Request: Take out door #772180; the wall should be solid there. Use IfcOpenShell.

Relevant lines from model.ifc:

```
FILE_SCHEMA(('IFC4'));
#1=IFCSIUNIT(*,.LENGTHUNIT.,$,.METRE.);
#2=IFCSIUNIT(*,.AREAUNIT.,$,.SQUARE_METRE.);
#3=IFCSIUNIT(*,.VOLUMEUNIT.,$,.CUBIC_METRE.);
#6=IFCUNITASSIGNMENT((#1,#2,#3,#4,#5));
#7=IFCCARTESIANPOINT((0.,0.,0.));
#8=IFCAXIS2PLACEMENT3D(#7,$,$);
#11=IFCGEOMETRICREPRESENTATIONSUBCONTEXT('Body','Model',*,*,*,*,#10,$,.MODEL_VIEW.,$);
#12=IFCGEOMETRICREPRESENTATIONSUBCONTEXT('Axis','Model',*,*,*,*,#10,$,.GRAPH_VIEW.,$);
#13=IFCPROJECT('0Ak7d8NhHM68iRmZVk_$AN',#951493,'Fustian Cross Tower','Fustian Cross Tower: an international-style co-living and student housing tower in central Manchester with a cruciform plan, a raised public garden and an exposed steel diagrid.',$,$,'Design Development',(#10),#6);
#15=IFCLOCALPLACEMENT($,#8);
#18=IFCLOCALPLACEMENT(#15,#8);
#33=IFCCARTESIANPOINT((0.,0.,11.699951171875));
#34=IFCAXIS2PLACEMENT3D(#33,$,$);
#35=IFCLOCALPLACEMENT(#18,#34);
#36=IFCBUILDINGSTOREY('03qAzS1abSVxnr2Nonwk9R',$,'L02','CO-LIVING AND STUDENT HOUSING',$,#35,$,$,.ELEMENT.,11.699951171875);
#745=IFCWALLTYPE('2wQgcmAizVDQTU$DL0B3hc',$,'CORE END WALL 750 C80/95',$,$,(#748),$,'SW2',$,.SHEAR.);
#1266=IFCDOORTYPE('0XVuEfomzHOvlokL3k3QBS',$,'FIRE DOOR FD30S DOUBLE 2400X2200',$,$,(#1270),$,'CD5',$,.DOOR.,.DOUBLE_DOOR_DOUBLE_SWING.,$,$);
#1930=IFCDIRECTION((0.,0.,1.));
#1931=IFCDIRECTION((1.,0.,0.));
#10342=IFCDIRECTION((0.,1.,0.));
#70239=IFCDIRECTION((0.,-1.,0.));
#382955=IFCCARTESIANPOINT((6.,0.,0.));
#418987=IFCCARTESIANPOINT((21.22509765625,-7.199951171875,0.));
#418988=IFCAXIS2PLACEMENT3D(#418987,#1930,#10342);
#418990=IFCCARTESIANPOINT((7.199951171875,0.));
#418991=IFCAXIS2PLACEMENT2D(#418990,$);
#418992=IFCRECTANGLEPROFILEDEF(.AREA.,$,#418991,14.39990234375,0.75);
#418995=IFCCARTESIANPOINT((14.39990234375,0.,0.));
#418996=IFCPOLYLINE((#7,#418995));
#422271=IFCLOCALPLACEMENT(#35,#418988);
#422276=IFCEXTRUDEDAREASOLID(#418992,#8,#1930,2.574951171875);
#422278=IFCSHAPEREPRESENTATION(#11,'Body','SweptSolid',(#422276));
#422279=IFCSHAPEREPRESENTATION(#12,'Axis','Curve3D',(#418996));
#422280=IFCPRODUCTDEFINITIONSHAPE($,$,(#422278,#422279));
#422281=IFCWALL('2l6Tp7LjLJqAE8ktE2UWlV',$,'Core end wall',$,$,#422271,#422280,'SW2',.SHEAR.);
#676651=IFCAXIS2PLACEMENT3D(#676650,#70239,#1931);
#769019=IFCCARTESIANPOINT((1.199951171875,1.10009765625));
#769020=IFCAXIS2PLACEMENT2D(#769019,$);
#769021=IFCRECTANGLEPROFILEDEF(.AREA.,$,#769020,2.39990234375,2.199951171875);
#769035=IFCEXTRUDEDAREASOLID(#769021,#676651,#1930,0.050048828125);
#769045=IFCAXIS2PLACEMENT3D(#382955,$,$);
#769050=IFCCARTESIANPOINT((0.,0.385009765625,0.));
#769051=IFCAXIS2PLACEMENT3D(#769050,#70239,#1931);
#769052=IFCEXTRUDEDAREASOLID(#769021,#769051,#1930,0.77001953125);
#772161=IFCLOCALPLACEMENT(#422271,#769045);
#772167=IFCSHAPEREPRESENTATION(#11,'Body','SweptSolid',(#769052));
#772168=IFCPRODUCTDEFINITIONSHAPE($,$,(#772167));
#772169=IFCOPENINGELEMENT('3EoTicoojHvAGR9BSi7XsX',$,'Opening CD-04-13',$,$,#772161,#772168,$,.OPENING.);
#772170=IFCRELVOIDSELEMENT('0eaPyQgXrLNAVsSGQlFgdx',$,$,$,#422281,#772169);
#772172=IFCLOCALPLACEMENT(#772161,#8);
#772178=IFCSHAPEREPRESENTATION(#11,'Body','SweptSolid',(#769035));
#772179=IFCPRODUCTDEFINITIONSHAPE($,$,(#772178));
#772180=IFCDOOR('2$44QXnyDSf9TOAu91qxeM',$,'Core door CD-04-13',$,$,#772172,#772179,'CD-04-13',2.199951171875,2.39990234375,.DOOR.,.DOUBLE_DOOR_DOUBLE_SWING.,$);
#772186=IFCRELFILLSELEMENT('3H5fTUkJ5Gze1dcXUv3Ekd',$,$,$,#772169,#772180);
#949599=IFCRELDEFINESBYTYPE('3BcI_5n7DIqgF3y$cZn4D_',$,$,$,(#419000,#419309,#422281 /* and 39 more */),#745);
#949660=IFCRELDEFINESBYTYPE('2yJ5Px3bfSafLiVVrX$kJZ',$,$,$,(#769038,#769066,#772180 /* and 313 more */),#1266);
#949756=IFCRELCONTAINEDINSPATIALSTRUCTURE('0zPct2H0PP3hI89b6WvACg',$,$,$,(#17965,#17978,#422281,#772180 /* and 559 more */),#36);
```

```python
import ifcopenshell
import ifcopenshell.api.feature
import ifcopenshell.api.root
import ifcopenshell.geom
import ifcopenshell.util.shape

model = ifcopenshell.open("model.ifc")
settings = ifcopenshell.geom.settings()


def volume(element):
    """Net volume in cubic metres, openings subtracted."""
    shape = ifcopenshell.geom.create_shape(settings, element)
    return ifcopenshell.util.shape.get_volume(shape.geometry)


door = model.by_guid("2$44QXnyDSf9TOAu91qxeM")
opening = door.FillsVoids[0].RelatingOpeningElement
wall = opening.VoidsElements[0].RelatingBuildingElement
before = volume(wall)

ifcopenshell.api.root.remove_product(model, product=door)
ifcopenshell.api.feature.remove_feature(model, feature=opening)

after = volume(wall)

print(f"wall volume {before:.3f} -> {after:.3f} m3")

model.write("model_updated.ifc")
```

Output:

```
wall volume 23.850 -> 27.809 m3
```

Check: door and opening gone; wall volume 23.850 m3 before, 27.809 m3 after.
